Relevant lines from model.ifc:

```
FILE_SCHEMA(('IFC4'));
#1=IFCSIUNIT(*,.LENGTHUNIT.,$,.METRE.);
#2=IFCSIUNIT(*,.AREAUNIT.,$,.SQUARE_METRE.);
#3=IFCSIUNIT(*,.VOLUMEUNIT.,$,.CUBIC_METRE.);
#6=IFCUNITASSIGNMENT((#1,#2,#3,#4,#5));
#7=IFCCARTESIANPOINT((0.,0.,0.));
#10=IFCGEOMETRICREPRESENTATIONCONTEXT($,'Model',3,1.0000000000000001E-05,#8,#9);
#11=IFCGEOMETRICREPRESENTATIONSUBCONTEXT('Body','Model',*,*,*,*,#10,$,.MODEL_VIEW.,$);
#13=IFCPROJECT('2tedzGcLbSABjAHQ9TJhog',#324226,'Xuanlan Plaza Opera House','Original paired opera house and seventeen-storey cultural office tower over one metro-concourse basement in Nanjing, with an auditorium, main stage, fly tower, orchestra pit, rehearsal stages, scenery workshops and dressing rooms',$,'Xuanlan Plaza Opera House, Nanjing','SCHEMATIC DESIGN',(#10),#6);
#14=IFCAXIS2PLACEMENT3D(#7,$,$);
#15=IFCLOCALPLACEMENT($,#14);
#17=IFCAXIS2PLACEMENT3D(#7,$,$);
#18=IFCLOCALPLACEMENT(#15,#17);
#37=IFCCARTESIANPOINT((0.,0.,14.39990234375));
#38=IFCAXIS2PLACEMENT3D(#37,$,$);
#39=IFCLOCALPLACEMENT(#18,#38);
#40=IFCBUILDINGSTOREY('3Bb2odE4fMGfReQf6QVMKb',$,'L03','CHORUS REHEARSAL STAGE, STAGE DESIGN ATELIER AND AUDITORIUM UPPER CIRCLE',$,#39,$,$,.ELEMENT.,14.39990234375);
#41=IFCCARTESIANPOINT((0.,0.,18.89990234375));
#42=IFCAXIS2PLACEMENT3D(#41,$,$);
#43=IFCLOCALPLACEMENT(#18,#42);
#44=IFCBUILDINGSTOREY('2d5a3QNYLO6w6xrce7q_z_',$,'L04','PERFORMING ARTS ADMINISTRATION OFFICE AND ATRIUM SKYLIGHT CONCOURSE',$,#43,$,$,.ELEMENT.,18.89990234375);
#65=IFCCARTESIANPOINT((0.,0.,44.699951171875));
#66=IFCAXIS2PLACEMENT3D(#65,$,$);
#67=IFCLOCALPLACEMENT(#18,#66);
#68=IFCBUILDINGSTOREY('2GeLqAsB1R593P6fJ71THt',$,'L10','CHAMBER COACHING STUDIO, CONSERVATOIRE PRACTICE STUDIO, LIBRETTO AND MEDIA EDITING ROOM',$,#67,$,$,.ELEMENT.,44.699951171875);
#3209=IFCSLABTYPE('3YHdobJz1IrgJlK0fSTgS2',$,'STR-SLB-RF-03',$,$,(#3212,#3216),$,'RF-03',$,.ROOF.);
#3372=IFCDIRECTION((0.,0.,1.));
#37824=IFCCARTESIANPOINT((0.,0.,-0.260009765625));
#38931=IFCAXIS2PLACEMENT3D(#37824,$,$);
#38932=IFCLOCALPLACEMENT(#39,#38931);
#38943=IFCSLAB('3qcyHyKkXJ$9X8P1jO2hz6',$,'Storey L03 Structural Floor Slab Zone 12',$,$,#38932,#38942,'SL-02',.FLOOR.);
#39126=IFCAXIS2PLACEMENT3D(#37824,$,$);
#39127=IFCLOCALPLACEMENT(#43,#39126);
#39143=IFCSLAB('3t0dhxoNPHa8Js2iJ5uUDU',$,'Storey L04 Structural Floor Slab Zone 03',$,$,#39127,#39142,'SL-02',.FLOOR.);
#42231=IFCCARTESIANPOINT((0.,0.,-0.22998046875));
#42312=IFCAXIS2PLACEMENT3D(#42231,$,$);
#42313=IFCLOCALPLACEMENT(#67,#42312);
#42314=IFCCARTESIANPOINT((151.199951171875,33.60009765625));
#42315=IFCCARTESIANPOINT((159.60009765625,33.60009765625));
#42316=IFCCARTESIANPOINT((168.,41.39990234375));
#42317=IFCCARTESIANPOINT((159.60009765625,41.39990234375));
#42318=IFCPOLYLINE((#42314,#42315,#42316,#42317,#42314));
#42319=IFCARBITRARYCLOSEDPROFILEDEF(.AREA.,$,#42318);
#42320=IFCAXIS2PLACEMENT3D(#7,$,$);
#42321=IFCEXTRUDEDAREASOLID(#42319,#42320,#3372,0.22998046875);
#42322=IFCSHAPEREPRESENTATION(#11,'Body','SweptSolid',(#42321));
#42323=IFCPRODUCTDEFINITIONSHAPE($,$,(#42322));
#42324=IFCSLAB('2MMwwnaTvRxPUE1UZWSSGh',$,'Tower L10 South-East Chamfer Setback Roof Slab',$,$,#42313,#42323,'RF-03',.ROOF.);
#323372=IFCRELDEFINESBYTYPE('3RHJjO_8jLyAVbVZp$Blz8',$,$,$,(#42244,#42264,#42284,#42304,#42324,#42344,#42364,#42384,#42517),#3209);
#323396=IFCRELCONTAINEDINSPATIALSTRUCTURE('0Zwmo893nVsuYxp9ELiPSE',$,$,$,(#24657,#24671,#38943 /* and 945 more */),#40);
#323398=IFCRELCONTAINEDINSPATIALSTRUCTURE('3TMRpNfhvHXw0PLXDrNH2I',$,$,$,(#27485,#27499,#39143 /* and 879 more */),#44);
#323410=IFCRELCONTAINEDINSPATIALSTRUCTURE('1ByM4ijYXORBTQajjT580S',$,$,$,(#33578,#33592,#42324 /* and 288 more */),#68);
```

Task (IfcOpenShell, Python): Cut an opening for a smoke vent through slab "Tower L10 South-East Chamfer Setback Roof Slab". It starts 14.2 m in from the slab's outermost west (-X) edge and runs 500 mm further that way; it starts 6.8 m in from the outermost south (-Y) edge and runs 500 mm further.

```python
import numpy as np
import ifcopenshell
import ifcopenshell.api.feature
import ifcopenshell.api.geometry
import ifcopenshell.api.root
import ifcopenshell.geom
import ifcopenshell.util.placement
import ifcopenshell.util.representation
import ifcopenshell.util.shape
import ifcopenshell.util.unit

model = ifcopenshell.open("model.ifc")
unit_scale = ifcopenshell.util.unit.calculate_unit_scale(model)
settings = ifcopenshell.geom.settings()


def volume(element):
    """Net volume in cubic metres, openings subtracted."""
    shape = ifcopenshell.geom.create_shape(settings, element)
    return ifcopenshell.util.shape.get_volume(shape.geometry)


slab = model.by_id(42324)
before = volume(slab)

# Extent in the slab's own axes, in metres. The edges named are its -X and -Y sides.
slab_shape = ifcopenshell.geom.create_shape(settings, slab)
vertices = ifcopenshell.util.shape.get_vertices(slab_shape.geometry)
x_min, y_min, bottom = vertices.min(axis=0)
top = vertices[:, 2].max()

opening = ifcopenshell.api.root.create_entity(model, ifc_class="IfcOpeningElement", name="Smoke vent opening", predefined_type="OPENING")
context = ifcopenshell.util.representation.get_context(model, "Model", "Body", "MODEL_VIEW")
width, depth = 0.5, 0.5
outline = [(0.0, 0.0), (width, 0.0), (width, depth), (0.0, depth), (0.0, 0.0)]
# Overshoot both faces by 50 mm so the cut is clean.
shape = ifcopenshell.api.geometry.add_slab_representation(
    model, context=context, depth=top - bottom + 0.1, polyline=outline
)
ifcopenshell.api.geometry.assign_representation(model, product=opening, representation=shape)

matrix = ifcopenshell.util.placement.get_local_placement(slab.ObjectPlacement)
matrix[:, 3] = matrix @ np.append(np.array([x_min + 14.2, y_min + 6.8, bottom - 0.05]) / unit_scale, 1.0)
ifcopenshell.api.geometry.edit_object_placement(model, product=opening, matrix=matrix, is_si=False)
ifcopenshell.api.feature.add_feature(model, feature=opening, element=slab)

after = volume(slab)

print(f"slab volume {before:.3f} -> {after:.3f} m3")

model.write("model_updated.ifc")
```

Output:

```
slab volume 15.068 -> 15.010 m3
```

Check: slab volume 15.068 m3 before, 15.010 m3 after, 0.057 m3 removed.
